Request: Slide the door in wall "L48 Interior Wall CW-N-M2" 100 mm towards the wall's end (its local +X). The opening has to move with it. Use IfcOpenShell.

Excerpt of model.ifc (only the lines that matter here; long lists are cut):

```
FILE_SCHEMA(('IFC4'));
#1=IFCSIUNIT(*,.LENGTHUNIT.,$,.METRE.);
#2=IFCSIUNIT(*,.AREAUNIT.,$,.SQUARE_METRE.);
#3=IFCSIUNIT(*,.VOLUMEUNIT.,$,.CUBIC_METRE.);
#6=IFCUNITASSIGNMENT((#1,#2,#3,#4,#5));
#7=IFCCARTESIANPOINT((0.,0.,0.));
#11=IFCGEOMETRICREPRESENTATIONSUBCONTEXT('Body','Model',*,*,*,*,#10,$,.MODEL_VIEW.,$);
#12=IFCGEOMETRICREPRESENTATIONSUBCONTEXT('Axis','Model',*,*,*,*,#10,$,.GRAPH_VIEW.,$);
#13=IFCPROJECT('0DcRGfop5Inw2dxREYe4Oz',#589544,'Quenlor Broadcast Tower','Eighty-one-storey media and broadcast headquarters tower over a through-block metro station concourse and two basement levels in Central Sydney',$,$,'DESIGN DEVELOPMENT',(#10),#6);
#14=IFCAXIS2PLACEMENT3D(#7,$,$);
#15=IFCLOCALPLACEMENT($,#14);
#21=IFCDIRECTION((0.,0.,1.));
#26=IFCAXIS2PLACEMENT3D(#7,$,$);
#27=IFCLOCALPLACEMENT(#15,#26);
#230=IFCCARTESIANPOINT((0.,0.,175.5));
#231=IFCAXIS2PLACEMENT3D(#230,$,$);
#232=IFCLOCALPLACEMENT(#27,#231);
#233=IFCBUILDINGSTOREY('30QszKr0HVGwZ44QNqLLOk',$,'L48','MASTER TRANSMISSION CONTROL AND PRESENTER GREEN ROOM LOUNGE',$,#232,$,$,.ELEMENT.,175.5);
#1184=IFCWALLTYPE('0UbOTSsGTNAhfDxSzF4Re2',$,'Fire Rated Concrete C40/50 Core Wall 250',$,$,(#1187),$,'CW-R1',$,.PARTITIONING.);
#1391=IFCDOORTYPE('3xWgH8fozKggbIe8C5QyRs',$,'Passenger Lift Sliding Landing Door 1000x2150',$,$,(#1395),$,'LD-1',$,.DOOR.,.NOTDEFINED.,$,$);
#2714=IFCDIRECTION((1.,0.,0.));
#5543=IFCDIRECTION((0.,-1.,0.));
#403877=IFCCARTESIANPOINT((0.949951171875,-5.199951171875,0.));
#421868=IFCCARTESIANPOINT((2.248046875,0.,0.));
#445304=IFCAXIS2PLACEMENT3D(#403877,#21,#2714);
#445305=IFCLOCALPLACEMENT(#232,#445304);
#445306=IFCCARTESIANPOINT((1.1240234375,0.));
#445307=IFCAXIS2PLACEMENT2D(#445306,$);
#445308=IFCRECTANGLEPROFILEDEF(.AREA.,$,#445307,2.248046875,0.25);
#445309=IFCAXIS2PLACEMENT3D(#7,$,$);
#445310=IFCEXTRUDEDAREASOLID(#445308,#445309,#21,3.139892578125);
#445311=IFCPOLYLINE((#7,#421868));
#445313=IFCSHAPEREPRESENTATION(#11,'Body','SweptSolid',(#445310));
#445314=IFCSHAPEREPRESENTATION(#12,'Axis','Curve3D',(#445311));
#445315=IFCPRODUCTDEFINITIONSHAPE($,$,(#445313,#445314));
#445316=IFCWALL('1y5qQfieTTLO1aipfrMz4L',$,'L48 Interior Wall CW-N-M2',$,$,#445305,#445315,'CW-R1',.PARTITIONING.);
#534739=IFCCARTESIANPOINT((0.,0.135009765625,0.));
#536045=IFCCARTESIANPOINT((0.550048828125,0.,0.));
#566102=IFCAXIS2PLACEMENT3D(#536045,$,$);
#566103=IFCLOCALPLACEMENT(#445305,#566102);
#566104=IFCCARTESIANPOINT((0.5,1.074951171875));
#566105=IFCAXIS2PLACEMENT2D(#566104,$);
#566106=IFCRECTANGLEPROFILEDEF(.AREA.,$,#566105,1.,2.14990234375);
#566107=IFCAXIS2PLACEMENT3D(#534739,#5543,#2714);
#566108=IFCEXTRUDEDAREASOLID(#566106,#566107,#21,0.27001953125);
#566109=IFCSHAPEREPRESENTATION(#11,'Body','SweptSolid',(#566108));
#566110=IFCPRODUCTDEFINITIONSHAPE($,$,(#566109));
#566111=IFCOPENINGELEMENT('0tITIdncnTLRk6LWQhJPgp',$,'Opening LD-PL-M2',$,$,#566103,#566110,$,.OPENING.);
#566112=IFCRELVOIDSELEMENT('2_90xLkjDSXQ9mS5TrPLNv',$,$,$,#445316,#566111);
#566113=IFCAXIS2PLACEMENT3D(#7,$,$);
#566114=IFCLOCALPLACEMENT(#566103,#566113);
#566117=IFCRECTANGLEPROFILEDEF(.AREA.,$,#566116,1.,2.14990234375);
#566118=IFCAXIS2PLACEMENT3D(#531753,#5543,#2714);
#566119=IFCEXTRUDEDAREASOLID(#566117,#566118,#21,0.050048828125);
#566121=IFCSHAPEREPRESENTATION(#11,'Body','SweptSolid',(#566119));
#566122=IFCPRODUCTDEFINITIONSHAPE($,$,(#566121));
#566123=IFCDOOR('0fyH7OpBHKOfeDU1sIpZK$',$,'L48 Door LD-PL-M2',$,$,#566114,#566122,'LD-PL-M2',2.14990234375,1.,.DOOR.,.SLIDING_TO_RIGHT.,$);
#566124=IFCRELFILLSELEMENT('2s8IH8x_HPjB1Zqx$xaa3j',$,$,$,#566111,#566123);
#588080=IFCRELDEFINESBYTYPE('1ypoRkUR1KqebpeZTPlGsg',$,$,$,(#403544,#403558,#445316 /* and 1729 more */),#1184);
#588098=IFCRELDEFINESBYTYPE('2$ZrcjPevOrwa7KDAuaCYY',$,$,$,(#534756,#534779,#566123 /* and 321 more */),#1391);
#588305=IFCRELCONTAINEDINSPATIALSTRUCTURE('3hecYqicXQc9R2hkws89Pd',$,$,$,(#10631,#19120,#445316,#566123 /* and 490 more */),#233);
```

```python
import ifcopenshell
import ifcopenshell.api.geometry
import ifcopenshell.util.placement
import ifcopenshell.util.unit

model = ifcopenshell.open("model.ifc")
unit_scale = ifcopenshell.util.unit.calculate_unit_scale(model)

door = model.by_guid("0fyH7OpBHKOfeDU1sIpZK$")
opening = door.FillsVoids[0].RelatingOpeningElement
wall = opening.VoidsElements[0].RelatingBuildingElement

wall_matrix = ifcopenshell.util.placement.get_local_placement(wall.ObjectPlacement)
shift = wall_matrix[:3, 0] * 0.1 / unit_scale
before = ifcopenshell.util.placement.get_local_placement(door.ObjectPlacement)[:3, 3].copy()

# The door is placed relative to its opening, so it follows when the opening moves.
matrix = ifcopenshell.util.placement.get_local_placement(opening.ObjectPlacement)
matrix[:3, 3] += shift
ifcopenshell.api.geometry.edit_object_placement(
    model, product=opening, matrix=matrix, is_si=False, should_transform_children=True
)

after = ifcopenshell.util.placement.get_local_placement(door.ObjectPlacement)[:3, 3]
print("door moved by", (after - before).round(3) + 0.0)

model.write("model_rev.ifc")
```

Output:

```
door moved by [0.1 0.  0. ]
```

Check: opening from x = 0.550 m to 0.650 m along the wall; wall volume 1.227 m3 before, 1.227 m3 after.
